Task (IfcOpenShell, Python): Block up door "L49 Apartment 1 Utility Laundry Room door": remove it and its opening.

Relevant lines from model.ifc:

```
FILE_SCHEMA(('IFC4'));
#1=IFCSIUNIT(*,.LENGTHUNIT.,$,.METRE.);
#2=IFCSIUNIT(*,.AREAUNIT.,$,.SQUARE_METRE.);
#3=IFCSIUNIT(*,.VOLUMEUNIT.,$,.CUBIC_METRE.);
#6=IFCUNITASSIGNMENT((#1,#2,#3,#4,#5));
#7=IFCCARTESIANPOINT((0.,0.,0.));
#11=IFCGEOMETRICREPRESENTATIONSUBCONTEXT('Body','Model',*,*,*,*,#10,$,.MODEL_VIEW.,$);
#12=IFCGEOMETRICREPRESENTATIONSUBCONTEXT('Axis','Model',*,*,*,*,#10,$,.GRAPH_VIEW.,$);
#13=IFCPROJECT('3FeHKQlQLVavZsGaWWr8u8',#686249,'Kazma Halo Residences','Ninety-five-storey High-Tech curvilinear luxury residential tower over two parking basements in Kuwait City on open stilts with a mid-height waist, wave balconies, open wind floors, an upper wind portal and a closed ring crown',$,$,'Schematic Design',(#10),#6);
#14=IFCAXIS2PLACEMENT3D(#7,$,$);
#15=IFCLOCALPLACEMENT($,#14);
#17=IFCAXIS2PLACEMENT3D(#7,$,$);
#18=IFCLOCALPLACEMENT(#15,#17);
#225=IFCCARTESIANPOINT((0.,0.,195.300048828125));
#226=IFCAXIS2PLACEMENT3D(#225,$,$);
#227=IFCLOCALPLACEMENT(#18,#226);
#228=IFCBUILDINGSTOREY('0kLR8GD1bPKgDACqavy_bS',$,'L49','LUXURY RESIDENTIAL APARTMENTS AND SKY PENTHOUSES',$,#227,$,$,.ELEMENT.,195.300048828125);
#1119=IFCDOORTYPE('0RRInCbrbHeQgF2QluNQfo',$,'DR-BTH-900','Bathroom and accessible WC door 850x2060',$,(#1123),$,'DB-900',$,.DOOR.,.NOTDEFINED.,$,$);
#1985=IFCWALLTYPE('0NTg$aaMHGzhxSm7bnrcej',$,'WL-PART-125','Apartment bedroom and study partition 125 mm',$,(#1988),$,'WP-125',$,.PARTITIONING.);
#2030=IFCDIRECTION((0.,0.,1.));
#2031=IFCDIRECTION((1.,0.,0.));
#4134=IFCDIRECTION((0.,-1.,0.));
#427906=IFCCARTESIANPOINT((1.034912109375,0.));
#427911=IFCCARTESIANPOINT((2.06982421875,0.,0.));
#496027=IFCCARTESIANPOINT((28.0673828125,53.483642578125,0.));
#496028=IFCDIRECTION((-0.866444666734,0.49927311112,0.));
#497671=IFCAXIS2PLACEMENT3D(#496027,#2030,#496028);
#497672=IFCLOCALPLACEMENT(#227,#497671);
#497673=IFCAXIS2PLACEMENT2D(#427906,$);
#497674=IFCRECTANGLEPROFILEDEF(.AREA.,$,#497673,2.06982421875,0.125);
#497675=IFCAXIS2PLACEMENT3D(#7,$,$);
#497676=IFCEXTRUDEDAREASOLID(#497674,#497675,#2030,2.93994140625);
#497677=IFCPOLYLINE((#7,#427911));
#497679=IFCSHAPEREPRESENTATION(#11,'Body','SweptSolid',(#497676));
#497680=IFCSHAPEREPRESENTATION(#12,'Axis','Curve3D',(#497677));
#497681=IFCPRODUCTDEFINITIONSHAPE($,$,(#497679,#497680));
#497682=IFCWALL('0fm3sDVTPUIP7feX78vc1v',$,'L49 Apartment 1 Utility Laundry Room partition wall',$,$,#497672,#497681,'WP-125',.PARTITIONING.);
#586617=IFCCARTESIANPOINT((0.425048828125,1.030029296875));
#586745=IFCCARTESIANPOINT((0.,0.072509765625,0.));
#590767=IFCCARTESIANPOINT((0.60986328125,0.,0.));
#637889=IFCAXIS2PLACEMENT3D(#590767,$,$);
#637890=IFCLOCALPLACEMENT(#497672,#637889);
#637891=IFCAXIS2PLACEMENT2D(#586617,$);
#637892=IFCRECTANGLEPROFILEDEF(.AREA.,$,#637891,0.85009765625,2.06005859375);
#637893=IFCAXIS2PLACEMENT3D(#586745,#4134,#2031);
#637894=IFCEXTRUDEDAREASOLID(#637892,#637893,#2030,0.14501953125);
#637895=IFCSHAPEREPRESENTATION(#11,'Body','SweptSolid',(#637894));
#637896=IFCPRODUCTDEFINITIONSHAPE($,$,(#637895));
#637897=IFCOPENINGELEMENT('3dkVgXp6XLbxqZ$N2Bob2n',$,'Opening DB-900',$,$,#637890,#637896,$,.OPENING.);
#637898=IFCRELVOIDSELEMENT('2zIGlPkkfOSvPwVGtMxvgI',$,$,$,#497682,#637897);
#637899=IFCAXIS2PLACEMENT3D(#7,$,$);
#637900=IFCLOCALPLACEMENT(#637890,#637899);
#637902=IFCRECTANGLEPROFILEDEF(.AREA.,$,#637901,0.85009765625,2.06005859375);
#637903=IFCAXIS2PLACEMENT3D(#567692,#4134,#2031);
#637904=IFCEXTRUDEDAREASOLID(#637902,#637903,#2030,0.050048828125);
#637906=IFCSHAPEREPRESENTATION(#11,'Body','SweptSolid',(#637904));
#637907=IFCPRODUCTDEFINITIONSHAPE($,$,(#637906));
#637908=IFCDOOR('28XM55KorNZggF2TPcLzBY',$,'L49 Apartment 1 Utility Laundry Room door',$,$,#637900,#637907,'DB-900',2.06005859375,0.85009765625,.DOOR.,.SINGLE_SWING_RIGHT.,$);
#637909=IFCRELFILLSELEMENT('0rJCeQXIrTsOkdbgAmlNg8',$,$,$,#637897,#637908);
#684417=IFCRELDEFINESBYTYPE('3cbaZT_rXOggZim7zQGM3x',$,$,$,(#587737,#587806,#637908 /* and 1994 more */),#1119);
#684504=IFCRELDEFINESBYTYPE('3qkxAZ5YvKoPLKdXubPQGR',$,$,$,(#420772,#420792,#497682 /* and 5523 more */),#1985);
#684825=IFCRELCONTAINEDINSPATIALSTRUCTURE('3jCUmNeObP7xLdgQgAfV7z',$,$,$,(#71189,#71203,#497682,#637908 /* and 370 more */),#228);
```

```python
import ifcopenshell
import ifcopenshell.api.feature
import ifcopenshell.api.root
import ifcopenshell.geom
import ifcopenshell.util.shape

model = ifcopenshell.open("model.ifc")
settings = ifcopenshell.geom.settings()


def volume(element):
    """Net volume in cubic metres, openings subtracted."""
    shape = ifcopenshell.geom.create_shape(settings, element)
    return ifcopenshell.util.shape.get_volume(shape.geometry)


door = model.by_id(637908)
opening = door.FillsVoids[0].RelatingOpeningElement
wall = opening.VoidsElements[0].RelatingBuildingElement
before = volume(wall)

ifcopenshell.api.root.remove_product(model, product=door)
ifcopenshell.api.feature.remove_feature(model, feature=opening)

after = volume(wall)

print(f"wall volume {before:.3f} -> {after:.3f} m3")

model.write("model_v2.ifc")
```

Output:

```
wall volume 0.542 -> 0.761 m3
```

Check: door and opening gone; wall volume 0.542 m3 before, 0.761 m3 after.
